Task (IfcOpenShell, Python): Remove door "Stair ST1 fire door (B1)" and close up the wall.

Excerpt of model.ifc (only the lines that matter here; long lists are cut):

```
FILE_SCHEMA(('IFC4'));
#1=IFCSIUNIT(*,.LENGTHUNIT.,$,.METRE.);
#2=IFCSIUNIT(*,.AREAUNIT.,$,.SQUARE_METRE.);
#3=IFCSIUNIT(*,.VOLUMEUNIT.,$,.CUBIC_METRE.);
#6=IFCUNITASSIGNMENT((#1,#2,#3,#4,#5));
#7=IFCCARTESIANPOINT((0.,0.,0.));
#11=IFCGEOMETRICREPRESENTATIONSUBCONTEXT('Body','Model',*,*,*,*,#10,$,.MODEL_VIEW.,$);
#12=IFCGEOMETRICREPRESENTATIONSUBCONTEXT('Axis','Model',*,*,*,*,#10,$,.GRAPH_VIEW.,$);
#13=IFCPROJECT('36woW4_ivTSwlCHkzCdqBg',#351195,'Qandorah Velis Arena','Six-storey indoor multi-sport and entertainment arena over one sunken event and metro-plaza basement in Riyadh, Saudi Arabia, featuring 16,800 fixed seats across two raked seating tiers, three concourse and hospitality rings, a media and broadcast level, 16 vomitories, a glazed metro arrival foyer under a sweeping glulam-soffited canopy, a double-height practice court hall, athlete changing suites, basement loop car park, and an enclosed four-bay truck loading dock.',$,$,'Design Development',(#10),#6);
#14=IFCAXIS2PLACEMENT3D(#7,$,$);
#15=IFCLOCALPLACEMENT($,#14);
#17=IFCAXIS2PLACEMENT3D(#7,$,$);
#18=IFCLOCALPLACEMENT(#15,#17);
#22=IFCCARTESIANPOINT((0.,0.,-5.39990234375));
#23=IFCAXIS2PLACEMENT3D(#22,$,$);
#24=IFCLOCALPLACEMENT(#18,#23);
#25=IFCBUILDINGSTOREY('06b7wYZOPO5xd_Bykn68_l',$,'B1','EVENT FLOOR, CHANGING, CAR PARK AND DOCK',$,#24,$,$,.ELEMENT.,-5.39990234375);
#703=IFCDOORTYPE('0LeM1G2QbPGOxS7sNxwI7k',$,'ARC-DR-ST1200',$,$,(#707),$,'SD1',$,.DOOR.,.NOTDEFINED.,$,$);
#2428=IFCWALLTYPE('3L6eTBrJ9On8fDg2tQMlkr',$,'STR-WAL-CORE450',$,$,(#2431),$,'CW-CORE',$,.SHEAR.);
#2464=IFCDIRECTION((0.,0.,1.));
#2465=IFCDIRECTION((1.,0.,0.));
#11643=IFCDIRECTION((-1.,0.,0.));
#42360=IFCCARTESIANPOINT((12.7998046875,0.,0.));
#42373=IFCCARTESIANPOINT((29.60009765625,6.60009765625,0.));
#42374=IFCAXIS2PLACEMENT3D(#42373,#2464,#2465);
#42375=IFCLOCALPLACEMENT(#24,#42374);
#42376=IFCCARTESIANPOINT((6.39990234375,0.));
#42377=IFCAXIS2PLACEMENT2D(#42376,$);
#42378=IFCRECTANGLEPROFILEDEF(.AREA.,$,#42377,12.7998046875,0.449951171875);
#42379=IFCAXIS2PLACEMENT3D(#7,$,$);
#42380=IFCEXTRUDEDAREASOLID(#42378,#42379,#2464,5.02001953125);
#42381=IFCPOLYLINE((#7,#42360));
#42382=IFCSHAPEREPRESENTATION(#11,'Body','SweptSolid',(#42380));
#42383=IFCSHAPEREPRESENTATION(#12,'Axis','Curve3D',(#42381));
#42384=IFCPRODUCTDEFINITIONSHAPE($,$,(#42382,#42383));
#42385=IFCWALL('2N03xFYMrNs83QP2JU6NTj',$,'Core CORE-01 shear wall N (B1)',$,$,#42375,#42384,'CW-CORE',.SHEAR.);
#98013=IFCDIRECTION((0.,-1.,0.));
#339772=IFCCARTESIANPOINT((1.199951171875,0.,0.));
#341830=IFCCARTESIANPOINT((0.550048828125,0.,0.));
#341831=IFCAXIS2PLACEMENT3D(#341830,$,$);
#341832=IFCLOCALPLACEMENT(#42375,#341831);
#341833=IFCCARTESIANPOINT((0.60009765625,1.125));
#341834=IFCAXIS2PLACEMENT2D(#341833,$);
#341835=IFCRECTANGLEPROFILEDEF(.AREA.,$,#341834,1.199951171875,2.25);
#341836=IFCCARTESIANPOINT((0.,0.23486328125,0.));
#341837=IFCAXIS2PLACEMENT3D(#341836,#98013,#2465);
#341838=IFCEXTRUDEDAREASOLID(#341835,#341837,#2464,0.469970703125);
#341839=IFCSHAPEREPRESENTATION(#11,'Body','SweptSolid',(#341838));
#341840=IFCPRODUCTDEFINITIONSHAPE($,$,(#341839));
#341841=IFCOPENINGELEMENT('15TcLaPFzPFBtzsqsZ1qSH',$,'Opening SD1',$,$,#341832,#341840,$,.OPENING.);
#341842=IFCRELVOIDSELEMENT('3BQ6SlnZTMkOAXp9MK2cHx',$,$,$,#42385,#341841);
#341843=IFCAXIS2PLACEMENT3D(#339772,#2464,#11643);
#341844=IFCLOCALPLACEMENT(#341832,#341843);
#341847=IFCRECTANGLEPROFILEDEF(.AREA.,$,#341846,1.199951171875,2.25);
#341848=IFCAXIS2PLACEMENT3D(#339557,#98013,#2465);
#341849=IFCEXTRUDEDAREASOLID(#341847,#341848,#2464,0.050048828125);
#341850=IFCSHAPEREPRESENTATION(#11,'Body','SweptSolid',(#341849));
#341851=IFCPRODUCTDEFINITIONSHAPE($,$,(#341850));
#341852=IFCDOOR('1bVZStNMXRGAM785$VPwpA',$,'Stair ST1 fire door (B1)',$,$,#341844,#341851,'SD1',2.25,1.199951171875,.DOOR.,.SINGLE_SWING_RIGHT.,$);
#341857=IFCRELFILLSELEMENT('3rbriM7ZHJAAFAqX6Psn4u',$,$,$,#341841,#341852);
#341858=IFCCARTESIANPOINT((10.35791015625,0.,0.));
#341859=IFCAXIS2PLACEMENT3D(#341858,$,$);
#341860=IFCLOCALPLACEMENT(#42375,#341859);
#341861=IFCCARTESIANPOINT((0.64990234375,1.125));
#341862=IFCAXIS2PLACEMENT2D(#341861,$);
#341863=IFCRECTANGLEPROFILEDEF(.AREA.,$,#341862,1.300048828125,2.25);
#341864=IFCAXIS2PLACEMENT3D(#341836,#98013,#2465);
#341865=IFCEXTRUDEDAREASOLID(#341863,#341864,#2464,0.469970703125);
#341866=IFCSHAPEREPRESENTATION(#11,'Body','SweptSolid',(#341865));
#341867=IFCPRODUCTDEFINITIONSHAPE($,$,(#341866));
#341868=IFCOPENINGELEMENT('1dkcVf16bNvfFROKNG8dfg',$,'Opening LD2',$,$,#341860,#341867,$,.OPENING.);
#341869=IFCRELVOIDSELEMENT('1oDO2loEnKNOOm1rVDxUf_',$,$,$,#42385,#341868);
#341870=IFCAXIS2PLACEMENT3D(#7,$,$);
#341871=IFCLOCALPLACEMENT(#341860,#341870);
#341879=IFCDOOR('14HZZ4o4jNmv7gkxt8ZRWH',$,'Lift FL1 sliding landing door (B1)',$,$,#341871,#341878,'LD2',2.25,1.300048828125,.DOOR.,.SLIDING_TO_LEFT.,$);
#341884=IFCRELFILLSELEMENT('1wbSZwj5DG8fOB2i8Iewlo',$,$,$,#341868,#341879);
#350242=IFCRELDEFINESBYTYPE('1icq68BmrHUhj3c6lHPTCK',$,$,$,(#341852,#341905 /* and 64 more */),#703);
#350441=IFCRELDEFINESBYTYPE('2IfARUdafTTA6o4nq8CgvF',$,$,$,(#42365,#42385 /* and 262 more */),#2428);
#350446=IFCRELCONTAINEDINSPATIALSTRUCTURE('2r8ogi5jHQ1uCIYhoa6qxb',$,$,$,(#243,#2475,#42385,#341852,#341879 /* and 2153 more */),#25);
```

```python
import ifcopenshell
import ifcopenshell.api.feature
import ifcopenshell.api.root
import ifcopenshell.geom
import ifcopenshell.util.shape

model = ifcopenshell.open("model.ifc")
settings = ifcopenshell.geom.settings()


def volume(element):
    """Net volume in cubic metres, openings subtracted."""
    shape = ifcopenshell.geom.create_shape(settings, element)
    return ifcopenshell.util.shape.get_volume(shape.geometry)


door = model.by_guid("1bVZStNMXRGAM785$VPwpA")
opening = door.FillsVoids[0].RelatingOpeningElement
wall = opening.VoidsElements[0].RelatingBuildingElement
before = volume(wall)

ifcopenshell.api.root.remove_product(model, product=door)
ifcopenshell.api.feature.remove_feature(model, feature=opening)

after = volume(wall)

print(f"wall volume {before:.3f} -> {after:.3f} m3")

model.write("model_v2.ifc")
```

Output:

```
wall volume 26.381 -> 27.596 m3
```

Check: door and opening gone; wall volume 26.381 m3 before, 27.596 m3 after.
